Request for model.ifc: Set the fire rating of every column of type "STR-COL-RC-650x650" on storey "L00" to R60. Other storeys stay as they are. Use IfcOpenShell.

First a look at what the model holds.

```python
import ifcopenshell
import ifcopenshell.util.element

model = ifcopenshell.open("model.ifc")
print(model.schema)
storey = next(s for s in model.by_type("IfcBuildingStorey") if s.Name == "L00")
columns = [e for e in ifcopenshell.util.element.get_decomposition(storey) if e.is_a("IfcColumn")]
seen = {}
for e in columns:
    element_type = ifcopenshell.util.element.get_type(e)
    key = (element_type.Name if element_type != e and element_type else None, ifcopenshell.util.element.get_pset(e, "Pset_ColumnCommon", "FireRating"))
    seen[key] = seen.get(key, 0) + 1
for (name, value), count in sorted(seen.items(), key=str):
    print(count, "x", name, "|", value)
```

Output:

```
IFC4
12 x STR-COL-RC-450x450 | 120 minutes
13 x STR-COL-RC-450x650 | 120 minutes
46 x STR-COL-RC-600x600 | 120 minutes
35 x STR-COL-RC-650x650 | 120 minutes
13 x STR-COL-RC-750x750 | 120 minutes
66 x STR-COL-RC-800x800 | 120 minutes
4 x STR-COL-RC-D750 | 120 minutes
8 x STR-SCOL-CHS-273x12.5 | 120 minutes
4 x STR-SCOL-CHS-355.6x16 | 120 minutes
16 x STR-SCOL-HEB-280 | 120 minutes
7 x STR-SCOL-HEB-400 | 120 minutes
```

```python
import ifcopenshell
import ifcopenshell.api.pset
import ifcopenshell.util.element

model = ifcopenshell.open("model.ifc")

storey = next(s for s in model.by_type("IfcBuildingStorey") if s.Name == "L00")
columns = [e for e in ifcopenshell.util.element.get_decomposition(storey) if e.is_a("IfcColumn")]

count = 0
for e in columns:
    element_type = ifcopenshell.util.element.get_type(e)
    if element_type in (None, e) or element_type.Name != "STR-COL-RC-650x650":
        continue
    # add_pset returns the element's existing set when there is one.
    pset = ifcopenshell.api.pset.add_pset(model, product=e, name="Pset_ColumnCommon")
    ifcopenshell.api.pset.edit_pset(model, pset=pset, properties={"FireRating": "R60"})
    count += 1

print(count, "columns updated")

model.write("model-out.ifc")
```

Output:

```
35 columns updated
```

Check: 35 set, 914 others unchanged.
